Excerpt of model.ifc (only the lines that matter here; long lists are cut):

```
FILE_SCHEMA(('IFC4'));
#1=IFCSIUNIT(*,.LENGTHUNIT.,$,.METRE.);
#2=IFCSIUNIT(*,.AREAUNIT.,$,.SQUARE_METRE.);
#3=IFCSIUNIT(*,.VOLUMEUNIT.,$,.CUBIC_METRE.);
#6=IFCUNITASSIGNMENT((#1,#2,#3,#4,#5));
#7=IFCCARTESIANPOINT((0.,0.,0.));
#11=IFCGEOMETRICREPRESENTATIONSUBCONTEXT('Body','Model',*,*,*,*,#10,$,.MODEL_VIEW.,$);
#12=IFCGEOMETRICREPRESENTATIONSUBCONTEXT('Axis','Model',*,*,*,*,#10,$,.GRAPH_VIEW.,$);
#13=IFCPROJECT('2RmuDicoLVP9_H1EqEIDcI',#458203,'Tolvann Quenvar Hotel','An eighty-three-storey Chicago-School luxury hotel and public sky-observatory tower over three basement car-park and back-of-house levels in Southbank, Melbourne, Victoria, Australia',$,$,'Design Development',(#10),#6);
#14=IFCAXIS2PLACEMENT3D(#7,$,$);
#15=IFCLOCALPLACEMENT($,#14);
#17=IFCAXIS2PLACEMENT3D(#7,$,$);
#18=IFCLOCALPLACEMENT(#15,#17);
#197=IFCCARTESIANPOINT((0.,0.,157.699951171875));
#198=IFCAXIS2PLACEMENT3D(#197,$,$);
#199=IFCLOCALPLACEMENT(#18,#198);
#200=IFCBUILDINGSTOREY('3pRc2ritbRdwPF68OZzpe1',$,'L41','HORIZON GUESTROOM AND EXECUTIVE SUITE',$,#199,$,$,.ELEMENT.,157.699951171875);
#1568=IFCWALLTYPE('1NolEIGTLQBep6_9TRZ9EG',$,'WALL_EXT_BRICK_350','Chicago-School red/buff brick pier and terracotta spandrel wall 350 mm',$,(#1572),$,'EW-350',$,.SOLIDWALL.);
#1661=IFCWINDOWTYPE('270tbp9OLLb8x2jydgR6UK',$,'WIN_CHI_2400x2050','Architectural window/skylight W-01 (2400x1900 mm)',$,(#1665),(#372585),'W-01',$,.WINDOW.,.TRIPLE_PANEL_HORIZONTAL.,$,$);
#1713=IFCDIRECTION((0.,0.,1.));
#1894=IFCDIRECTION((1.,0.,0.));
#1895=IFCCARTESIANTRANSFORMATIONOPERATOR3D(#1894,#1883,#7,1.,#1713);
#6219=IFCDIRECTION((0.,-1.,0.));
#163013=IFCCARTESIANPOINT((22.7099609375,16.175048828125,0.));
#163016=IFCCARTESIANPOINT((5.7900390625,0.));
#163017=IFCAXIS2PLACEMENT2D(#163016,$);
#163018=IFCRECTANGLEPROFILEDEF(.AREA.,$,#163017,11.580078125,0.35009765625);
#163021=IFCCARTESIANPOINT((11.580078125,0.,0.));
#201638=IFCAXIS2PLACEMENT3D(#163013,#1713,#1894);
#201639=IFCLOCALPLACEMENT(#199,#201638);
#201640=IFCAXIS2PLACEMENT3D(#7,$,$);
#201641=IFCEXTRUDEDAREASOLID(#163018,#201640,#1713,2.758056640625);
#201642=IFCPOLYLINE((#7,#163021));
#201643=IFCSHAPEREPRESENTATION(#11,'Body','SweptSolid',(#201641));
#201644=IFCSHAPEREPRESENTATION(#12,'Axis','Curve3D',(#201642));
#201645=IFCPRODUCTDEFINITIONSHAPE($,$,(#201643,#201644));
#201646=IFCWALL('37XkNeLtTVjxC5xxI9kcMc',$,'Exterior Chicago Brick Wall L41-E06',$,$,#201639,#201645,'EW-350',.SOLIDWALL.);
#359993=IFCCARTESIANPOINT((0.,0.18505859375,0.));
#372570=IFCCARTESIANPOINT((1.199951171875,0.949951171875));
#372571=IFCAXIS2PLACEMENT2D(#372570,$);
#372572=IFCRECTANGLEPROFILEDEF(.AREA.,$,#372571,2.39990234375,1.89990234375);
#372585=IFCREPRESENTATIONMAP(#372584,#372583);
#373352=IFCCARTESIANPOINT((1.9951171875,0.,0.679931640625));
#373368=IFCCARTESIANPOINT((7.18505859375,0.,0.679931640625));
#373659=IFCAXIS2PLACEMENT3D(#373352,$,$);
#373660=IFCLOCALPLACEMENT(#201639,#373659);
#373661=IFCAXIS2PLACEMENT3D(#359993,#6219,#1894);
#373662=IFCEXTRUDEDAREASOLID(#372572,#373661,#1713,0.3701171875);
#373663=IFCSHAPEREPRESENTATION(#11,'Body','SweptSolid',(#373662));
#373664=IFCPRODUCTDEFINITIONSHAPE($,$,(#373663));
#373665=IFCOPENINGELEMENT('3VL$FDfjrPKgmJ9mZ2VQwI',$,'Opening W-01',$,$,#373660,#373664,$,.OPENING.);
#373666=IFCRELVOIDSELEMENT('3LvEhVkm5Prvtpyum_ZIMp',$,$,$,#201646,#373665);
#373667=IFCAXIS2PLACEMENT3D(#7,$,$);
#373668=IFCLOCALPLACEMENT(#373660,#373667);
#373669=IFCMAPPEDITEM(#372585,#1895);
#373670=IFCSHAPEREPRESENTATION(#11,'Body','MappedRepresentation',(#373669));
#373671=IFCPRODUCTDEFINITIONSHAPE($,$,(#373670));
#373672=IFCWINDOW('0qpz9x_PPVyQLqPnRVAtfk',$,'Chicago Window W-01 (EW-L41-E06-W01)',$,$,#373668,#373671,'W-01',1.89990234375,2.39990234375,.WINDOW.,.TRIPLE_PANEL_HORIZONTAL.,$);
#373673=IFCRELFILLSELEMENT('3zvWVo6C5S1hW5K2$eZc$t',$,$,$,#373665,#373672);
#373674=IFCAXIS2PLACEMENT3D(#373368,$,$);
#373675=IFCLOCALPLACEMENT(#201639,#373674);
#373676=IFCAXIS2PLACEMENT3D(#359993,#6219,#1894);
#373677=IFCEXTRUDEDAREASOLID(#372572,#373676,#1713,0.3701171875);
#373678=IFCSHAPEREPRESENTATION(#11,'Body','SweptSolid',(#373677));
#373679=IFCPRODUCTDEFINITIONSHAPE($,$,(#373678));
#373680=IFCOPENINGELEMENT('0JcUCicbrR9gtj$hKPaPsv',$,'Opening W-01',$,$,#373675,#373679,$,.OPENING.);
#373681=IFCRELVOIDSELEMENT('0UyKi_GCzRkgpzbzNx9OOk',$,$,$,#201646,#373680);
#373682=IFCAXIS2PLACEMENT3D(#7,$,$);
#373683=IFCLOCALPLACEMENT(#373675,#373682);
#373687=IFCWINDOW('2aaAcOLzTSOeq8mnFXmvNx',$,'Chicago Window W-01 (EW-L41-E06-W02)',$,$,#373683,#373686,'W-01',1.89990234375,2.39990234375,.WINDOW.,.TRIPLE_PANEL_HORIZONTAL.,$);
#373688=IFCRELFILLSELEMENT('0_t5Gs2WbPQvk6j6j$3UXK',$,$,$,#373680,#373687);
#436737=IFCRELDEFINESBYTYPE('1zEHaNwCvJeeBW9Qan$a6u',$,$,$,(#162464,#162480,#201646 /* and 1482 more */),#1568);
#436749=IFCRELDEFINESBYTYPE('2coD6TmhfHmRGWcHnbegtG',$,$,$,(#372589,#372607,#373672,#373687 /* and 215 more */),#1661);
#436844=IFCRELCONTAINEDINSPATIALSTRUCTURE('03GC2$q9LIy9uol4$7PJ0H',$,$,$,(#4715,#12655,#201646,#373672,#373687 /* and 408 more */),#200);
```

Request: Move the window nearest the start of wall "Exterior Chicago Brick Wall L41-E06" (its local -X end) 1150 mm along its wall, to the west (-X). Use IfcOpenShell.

```python
import ifcopenshell
import ifcopenshell.api.geometry
import ifcopenshell.util.placement
import ifcopenshell.util.unit

model = ifcopenshell.open("model.ifc")
unit_scale = ifcopenshell.util.unit.calculate_unit_scale(model)

window = model.by_guid("0qpz9x_PPVyQLqPnRVAtfk")
opening = window.FillsVoids[0].RelatingOpeningElement
wall = opening.VoidsElements[0].RelatingBuildingElement

wall_matrix = ifcopenshell.util.placement.get_local_placement(wall.ObjectPlacement)
shift = wall_matrix[:3, 0] * -1.15 / unit_scale
before = ifcopenshell.util.placement.get_local_placement(window.ObjectPlacement)[:3, 3].copy()

# The window is placed relative to its opening, so it follows when the opening moves.
matrix = ifcopenshell.util.placement.get_local_placement(opening.ObjectPlacement)
matrix[:3, 3] += shift
ifcopenshell.api.geometry.edit_object_placement(
    model, product=opening, matrix=matrix, is_si=False, should_transform_children=True
)

after = ifcopenshell.util.placement.get_local_placement(window.ObjectPlacement)[:3, 3]
print("window moved by", (after - before).round(3) + 0.0)

model.write("model-out.ifc")
```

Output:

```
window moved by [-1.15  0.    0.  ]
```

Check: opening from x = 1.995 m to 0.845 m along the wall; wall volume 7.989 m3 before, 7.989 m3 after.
